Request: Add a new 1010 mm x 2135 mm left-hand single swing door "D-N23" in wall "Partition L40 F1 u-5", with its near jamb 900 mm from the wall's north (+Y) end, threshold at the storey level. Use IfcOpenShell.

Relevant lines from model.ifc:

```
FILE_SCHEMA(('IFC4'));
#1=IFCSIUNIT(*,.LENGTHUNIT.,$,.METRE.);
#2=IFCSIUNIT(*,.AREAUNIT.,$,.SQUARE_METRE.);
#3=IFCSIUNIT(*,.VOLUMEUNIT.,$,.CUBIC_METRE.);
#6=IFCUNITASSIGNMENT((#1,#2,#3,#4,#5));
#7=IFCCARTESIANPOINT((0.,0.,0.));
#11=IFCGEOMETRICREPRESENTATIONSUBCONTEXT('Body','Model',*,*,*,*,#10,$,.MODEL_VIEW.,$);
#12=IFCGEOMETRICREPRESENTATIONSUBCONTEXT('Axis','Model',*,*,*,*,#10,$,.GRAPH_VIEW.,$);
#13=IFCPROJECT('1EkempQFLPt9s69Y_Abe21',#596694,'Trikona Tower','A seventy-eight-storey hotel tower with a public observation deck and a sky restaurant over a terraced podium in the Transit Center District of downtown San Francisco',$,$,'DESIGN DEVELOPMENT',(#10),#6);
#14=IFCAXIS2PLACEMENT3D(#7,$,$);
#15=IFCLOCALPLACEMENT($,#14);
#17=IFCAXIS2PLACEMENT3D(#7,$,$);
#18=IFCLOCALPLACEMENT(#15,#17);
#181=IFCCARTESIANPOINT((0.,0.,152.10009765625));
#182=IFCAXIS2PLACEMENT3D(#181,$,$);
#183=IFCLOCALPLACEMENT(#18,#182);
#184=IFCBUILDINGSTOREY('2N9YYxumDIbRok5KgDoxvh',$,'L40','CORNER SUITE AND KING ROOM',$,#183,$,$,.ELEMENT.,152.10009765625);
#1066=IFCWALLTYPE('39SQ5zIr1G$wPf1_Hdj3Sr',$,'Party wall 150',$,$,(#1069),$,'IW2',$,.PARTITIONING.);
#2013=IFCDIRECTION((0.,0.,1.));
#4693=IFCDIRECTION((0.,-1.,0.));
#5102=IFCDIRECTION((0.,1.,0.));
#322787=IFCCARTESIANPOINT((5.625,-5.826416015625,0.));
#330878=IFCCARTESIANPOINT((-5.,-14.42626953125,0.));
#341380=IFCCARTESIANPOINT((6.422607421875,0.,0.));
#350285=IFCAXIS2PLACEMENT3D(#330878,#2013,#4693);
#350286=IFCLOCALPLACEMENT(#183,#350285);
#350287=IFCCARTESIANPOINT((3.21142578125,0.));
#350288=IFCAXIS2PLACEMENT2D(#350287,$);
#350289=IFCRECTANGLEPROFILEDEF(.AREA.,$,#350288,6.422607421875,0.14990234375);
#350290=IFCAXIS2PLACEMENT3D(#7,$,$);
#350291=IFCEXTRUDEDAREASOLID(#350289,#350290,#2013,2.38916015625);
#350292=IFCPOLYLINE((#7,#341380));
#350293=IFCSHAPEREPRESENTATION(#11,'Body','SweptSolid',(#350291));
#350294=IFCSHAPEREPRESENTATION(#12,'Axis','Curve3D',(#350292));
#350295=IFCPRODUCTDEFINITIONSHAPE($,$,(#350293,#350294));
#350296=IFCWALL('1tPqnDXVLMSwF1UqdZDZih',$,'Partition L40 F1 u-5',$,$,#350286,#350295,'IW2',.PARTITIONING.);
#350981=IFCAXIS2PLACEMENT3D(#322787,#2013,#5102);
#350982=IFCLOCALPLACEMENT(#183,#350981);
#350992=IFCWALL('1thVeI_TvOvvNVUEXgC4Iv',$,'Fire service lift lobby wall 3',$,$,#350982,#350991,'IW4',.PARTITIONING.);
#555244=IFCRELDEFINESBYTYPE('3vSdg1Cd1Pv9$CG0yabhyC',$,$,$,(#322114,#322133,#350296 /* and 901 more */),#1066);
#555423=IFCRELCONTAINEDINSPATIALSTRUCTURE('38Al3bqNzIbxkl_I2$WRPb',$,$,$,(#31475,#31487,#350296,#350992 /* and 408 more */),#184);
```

```python
import numpy as np
import ifcopenshell
import ifcopenshell.api.feature
import ifcopenshell.api.geometry
import ifcopenshell.api.root
import ifcopenshell.api.spatial
import ifcopenshell.geom
import ifcopenshell.util.element
import ifcopenshell.util.placement
import ifcopenshell.util.representation
import ifcopenshell.util.shape
import ifcopenshell.util.unit

model = ifcopenshell.open("model.ifc")
unit_scale = ifcopenshell.util.unit.calculate_unit_scale(model)
settings = ifcopenshell.geom.settings()


def volume(element):
    """Net volume in cubic metres, openings subtracted."""
    shape = ifcopenshell.geom.create_shape(settings, element)
    return ifcopenshell.util.shape.get_volume(shape.geometry)


wall = model.by_guid("1tPqnDXVLMSwF1UqdZDZih")
storey = ifcopenshell.util.element.get_container(wall, ifc_class="IfcBuildingStorey")
context = ifcopenshell.util.representation.get_context(model, "Model", "Body", "MODEL_VIEW")
before = volume(wall)

width, height, from_end, sill = 1.01, 2.135, 0.9, 0.0  # metres

# The wall runs along its own X axis, and the end named is its -X end.
wall_shape = ifcopenshell.geom.create_shape(settings, wall)
x, y, z = ifcopenshell.util.shape.get_vertices(wall_shape.geometry).T
start = x.min() + from_end
face, thickness = float(y.min()), float(y.max() - y.min())
wall_matrix = ifcopenshell.util.placement.get_local_placement(wall.ObjectPlacement)
level = ifcopenshell.util.placement.get_local_placement(storey.ObjectPlacement)[2, 3]


def in_wall(x, y):
    """Placement at x, y metres in the wall's axes, at sill height."""
    matrix = wall_matrix.copy()
    matrix[:, 3] = wall_matrix @ np.array([x / unit_scale, y / unit_scale, 0.0, 1.0])
    matrix[2, 3] = level + sill / unit_scale
    return matrix


# Opening: a box that overshoots both wall faces by 50 mm.
opening = ifcopenshell.api.root.create_entity(model, ifc_class="IfcOpeningElement", predefined_type="OPENING")
box = ifcopenshell.api.geometry.add_wall_representation(
    model, context=context, length=width, height=height, thickness=thickness + 0.1
)
ifcopenshell.api.geometry.assign_representation(model, product=opening, representation=box)
ifcopenshell.api.geometry.edit_object_placement(model, product=opening, matrix=in_wall(start, face - 0.05), is_si=False)
ifcopenshell.api.feature.add_feature(model, feature=opening, element=wall)

door = ifcopenshell.api.root.create_entity(model, ifc_class="IfcDoor", name="D-N23", predefined_type="DOOR")
door.OverallWidth, door.OverallHeight = width / unit_scale, height / unit_scale
door.OperationType = "SINGLE_SWING_LEFT"
body = ifcopenshell.api.geometry.add_door_representation(
    model,
    context=context,
    overall_width=door.OverallWidth,
    overall_height=door.OverallHeight,
    operation_type="SINGLE_SWING_LEFT",
    lining_properties={"LiningDepth": thickness / unit_scale, "ThresholdDepth": thickness / unit_scale},
)
ifcopenshell.api.geometry.assign_representation(model, product=door, representation=body)
ifcopenshell.api.spatial.assign_container(model, products=[door], relating_structure=storey)
ifcopenshell.api.feature.add_filling(model, opening=opening, element=door)

# The lining spans the wall, so the door starts at the wall face.
ifcopenshell.api.geometry.edit_object_placement(model, product=door, matrix=in_wall(start, face), is_si=False)

after = volume(wall)

print(f"wall volume {before:.3f} -> {after:.3f} m3")

model.write("model_rev.ifc")
```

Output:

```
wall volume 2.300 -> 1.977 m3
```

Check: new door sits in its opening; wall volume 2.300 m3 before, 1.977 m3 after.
